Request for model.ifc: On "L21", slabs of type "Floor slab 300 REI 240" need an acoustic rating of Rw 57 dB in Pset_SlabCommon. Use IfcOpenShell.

First a look at what the model holds.

```python
import ifcopenshell
import ifcopenshell.util.element

model = ifcopenshell.open("model.ifc")
print(model.schema)
storey = next(s for s in model.by_type("IfcBuildingStorey") if s.Name == "L21")
slabs = [e for e in ifcopenshell.util.element.get_decomposition(storey) if e.is_a("IfcSlab")]
seen = {}
for e in slabs:
    element_type = ifcopenshell.util.element.get_type(e)
    key = (element_type.Name if element_type != e and element_type else None, ifcopenshell.util.element.get_pset(e, "Pset_SlabCommon", "AcousticRating"))
    seen[key] = seen.get(key, 0) + 1
for (name, value), count in sorted(seen.items(), key=str):
    print(count, "x", name, "|", value)
```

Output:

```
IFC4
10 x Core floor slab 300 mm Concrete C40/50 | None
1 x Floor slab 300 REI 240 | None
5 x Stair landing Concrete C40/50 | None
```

```python
import ifcopenshell
import ifcopenshell.api.pset
import ifcopenshell.util.element

model = ifcopenshell.open("model.ifc")

storey = next(s for s in model.by_type("IfcBuildingStorey") if s.Name == "L21")
slabs = [e for e in ifcopenshell.util.element.get_decomposition(storey) if e.is_a("IfcSlab")]

count = 0
for e in slabs:
    element_type = ifcopenshell.util.element.get_type(e)
    if element_type in (None, e) or element_type.Name != "Floor slab 300 REI 240":
        continue
    found = ifcopenshell.util.element.get_pset(e, "Pset_SlabCommon", should_inherit=False)
    if found:
        pset = model.by_id(found["id"])
        if len(ifcopenshell.util.element.get_elements_by_pset(pset)) > 1:
            pset = ifcopenshell.api.pset.unshare_pset(model, products=[e], pset=pset)[0]
    else:
        pset = ifcopenshell.api.pset.add_pset(model, product=e, name="Pset_SlabCommon")
    ifcopenshell.api.pset.edit_pset(model, pset=pset, properties={"AcousticRating": "Rw 57 dB"})
    count += 1

print(count, "slabs updated")

model.write("model_updated.ifc")
```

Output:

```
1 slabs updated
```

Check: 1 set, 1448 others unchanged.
